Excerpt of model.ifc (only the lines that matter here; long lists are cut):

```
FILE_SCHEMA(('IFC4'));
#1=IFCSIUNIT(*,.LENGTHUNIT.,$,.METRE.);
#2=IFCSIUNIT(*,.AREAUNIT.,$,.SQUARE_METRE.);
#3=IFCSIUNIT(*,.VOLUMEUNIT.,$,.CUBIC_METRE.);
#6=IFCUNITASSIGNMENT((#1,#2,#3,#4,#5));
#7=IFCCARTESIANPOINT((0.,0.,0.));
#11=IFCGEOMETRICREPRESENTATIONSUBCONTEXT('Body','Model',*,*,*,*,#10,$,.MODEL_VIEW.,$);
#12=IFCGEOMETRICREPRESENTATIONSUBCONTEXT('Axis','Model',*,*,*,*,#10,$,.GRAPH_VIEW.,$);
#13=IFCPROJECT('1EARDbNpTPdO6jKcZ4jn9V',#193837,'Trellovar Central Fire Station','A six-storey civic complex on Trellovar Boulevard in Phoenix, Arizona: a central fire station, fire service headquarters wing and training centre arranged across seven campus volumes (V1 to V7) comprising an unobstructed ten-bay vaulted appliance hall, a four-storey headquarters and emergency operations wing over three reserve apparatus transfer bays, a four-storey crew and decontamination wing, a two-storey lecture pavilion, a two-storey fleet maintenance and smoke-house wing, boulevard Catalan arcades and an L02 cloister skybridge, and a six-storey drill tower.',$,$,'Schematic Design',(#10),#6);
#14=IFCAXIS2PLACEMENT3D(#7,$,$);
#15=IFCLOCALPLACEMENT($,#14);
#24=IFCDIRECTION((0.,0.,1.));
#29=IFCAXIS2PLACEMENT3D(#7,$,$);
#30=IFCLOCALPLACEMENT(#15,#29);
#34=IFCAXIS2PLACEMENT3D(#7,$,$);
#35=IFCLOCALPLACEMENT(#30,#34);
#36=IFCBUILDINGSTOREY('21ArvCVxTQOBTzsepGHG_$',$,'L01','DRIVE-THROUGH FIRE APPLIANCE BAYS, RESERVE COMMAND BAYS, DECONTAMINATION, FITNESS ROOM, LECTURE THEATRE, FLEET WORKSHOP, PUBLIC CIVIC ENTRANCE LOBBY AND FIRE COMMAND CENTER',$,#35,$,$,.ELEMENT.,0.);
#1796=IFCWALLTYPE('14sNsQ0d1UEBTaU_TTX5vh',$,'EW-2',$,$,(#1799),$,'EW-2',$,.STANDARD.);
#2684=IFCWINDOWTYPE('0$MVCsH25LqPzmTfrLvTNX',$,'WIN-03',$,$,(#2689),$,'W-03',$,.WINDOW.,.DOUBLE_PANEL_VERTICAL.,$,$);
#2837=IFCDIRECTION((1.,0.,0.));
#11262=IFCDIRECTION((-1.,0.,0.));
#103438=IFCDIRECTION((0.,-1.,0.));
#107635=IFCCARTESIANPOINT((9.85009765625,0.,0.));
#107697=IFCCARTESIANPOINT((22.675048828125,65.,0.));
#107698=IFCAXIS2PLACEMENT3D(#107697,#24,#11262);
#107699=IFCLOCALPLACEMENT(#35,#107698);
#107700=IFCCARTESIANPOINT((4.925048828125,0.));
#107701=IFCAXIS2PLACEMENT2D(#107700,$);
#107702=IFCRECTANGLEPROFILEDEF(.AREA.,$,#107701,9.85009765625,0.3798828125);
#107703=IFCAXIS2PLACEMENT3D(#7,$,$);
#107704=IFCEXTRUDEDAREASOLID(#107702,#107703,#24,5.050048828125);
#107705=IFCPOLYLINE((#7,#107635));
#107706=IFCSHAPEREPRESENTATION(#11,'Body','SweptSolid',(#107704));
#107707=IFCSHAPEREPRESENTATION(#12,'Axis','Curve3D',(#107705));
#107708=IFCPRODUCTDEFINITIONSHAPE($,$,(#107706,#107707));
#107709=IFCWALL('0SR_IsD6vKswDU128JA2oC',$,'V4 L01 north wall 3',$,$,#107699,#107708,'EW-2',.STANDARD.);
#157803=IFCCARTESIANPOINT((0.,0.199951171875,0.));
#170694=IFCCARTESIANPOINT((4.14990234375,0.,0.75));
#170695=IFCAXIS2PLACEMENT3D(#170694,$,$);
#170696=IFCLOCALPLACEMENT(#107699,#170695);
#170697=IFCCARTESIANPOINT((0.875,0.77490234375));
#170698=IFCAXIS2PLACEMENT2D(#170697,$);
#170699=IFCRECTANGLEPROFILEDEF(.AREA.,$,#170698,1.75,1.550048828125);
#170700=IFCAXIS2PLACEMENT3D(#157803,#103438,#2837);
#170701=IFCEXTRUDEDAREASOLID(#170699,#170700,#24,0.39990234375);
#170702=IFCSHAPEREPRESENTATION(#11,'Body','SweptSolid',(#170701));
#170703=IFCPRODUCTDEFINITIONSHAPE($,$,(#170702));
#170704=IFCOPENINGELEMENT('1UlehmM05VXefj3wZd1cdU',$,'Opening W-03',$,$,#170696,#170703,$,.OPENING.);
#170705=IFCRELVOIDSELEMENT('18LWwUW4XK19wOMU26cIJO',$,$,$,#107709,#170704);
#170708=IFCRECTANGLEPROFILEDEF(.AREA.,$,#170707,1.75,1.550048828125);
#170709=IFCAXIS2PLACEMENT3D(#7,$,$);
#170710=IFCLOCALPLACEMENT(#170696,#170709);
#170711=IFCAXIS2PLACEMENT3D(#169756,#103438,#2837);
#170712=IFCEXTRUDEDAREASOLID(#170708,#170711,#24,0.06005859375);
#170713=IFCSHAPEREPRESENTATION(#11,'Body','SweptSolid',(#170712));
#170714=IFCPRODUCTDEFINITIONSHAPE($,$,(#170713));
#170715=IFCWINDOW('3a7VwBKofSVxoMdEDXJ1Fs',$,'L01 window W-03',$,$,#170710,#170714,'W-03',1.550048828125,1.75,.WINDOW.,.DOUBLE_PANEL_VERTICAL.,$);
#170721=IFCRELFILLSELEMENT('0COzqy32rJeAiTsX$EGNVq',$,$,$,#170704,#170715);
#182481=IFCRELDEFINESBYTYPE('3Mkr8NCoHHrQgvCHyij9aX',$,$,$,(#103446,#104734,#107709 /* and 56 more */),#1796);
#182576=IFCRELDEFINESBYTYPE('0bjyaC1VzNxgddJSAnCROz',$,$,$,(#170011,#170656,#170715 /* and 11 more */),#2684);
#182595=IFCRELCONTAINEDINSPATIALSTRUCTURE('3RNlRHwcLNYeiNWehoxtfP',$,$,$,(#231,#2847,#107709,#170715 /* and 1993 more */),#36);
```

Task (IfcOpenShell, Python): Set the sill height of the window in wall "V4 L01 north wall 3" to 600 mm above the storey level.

```python
import numpy as np
import ifcopenshell
import ifcopenshell.api.geometry
import ifcopenshell.geom
import ifcopenshell.util.element
import ifcopenshell.util.placement
import ifcopenshell.util.shape
import ifcopenshell.util.unit

model = ifcopenshell.open("model.ifc")
unit_scale = ifcopenshell.util.unit.calculate_unit_scale(model)

window = model.by_guid("3a7VwBKofSVxoMdEDXJ1Fs")
opening = window.FillsVoids[0].RelatingOpeningElement
storey = ifcopenshell.util.element.get_container(window, ifc_class="IfcBuildingStorey")
level = ifcopenshell.util.placement.get_local_placement(storey.ObjectPlacement)[2, 3]

# The opening's origin need not be at the sill, so measure its lowest point.
shape = ifcopenshell.geom.create_shape(ifcopenshell.geom.settings(), opening)
bottom = ifcopenshell.util.shape.get_shape_bottom_elevation(shape, shape.geometry) / unit_scale
dz = level + 0.6 / unit_scale - bottom

shift = np.array([0.0, 0.0, dz])
# The window is placed relative to its opening, so it follows when the opening moves.
matrix = ifcopenshell.util.placement.get_local_placement(opening.ObjectPlacement)
matrix[:3, 3] += shift
ifcopenshell.api.geometry.edit_object_placement(
    model, product=opening, matrix=matrix, is_si=False, should_transform_children=True
)

print(f"moved by {dz * unit_scale:+.3f} m")

model.write("model_v2.ifc")
```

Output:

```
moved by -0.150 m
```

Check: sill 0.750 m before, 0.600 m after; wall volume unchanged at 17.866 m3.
